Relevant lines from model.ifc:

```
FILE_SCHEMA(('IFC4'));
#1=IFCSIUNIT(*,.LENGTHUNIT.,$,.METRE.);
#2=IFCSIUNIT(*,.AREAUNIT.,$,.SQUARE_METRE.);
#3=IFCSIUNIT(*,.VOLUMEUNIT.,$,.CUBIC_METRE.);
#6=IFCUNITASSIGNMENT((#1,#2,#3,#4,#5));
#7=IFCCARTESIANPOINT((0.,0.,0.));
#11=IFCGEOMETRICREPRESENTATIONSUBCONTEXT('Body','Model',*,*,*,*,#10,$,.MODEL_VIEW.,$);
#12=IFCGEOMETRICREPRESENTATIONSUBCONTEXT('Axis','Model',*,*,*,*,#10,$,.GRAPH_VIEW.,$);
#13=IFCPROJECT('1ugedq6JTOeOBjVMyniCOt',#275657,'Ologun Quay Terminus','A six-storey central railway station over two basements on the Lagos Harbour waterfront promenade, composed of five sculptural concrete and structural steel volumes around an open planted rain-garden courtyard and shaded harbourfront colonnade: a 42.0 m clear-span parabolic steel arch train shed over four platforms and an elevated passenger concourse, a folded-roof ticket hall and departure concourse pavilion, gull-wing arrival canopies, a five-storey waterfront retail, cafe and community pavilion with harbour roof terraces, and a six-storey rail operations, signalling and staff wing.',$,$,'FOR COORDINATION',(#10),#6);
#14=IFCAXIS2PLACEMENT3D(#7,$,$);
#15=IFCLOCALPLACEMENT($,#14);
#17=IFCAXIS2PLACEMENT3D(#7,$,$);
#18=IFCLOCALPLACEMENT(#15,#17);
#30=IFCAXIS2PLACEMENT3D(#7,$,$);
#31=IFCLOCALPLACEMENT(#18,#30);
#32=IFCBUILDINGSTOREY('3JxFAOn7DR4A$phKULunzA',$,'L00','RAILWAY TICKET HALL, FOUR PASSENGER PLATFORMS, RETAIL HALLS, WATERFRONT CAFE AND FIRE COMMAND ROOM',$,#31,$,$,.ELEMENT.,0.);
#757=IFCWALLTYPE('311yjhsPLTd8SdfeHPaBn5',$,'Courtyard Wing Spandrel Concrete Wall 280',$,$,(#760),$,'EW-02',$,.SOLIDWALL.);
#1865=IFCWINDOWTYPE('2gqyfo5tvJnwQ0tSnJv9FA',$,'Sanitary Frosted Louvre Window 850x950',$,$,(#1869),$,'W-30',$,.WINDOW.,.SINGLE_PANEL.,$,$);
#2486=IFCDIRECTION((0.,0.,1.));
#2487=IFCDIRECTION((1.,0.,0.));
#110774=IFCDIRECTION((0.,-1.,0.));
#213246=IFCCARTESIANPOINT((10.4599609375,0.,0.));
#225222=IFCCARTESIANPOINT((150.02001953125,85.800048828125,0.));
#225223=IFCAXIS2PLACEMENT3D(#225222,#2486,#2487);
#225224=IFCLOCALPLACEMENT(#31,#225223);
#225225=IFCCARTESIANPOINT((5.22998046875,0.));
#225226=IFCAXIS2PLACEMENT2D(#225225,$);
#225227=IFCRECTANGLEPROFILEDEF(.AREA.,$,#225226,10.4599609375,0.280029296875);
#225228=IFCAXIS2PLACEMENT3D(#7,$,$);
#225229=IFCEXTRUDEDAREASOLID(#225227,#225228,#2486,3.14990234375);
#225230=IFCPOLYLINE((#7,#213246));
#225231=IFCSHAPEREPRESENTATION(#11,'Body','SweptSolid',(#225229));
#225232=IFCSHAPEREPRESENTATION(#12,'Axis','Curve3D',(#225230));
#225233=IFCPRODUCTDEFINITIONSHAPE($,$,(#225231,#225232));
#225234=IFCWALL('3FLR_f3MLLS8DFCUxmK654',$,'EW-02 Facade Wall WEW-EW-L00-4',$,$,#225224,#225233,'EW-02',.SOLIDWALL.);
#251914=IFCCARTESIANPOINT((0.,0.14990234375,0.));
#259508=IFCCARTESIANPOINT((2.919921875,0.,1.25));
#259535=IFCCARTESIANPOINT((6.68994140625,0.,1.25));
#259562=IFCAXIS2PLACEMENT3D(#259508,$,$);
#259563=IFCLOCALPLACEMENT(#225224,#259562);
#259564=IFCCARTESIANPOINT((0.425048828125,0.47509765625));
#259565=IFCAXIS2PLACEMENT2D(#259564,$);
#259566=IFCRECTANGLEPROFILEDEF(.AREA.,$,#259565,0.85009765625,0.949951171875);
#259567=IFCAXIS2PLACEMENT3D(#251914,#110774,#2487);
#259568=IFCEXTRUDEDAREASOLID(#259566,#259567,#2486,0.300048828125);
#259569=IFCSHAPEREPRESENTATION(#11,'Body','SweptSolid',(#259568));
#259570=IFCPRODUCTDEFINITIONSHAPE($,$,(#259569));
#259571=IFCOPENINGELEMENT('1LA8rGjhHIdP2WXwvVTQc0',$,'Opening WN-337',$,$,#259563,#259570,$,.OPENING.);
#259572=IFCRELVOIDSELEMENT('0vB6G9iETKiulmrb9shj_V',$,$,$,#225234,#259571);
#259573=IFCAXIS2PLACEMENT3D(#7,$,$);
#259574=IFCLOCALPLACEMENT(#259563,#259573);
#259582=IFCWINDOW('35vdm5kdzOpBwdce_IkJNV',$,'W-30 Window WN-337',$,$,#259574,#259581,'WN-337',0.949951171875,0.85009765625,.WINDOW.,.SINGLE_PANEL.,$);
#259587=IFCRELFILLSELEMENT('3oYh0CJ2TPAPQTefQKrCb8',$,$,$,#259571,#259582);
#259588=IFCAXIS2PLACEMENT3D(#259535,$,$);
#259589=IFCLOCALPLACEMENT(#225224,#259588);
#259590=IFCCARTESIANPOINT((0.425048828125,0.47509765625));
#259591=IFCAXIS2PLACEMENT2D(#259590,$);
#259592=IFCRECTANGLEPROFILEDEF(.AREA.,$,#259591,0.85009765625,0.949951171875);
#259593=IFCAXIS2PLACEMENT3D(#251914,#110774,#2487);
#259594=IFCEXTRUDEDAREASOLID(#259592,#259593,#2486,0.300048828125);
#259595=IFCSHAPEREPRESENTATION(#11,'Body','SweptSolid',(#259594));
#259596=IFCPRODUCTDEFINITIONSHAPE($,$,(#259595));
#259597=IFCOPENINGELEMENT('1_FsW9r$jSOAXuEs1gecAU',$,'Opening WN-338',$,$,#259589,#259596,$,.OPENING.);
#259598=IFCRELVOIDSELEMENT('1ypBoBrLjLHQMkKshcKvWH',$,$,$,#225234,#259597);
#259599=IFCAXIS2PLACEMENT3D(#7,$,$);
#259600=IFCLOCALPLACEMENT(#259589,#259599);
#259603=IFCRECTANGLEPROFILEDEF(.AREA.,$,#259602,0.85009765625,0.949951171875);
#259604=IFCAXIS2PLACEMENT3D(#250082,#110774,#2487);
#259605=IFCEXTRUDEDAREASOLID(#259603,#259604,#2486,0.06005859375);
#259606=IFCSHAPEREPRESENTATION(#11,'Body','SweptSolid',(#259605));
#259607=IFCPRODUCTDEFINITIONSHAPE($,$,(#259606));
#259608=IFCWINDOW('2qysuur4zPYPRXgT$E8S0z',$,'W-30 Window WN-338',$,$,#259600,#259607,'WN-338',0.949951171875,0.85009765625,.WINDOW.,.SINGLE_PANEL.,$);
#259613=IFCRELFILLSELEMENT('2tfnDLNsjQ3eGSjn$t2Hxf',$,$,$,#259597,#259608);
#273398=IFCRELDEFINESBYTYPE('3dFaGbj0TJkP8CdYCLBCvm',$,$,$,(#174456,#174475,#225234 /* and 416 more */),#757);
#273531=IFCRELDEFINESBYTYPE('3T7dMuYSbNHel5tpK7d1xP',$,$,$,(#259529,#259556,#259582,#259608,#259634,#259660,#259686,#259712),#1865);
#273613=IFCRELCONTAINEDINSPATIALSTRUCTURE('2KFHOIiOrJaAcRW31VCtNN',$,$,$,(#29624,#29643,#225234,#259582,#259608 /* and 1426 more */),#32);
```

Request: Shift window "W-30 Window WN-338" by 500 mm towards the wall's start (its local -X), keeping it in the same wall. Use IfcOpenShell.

```python
import ifcopenshell
import ifcopenshell.api.geometry
import ifcopenshell.util.placement

model = ifcopenshell.open("model.ifc")

window = model.by_id(259608)
opening = window.FillsVoids[0].RelatingOpeningElement
wall = opening.VoidsElements[0].RelatingBuildingElement

wall_matrix = ifcopenshell.util.placement.get_local_placement(wall.ObjectPlacement)
shift = wall_matrix[:3, 0] * -0.5
before = ifcopenshell.util.placement.get_local_placement(window.ObjectPlacement)[:3, 3].copy()

# The window is placed relative to its opening, so it follows when the opening moves.
matrix = ifcopenshell.util.placement.get_local_placement(opening.ObjectPlacement)
matrix[:3, 3] += shift
ifcopenshell.api.geometry.edit_object_placement(
    model, product=opening, matrix=matrix, is_si=False, should_transform_children=True
)

after = ifcopenshell.util.placement.get_local_placement(window.ObjectPlacement)[:3, 3]
print("window moved by", (after - before).round(3) + 0.0)

model.write("model_updated.ifc")
```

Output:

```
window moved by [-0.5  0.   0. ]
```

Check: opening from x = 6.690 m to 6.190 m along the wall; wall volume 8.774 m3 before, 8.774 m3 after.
